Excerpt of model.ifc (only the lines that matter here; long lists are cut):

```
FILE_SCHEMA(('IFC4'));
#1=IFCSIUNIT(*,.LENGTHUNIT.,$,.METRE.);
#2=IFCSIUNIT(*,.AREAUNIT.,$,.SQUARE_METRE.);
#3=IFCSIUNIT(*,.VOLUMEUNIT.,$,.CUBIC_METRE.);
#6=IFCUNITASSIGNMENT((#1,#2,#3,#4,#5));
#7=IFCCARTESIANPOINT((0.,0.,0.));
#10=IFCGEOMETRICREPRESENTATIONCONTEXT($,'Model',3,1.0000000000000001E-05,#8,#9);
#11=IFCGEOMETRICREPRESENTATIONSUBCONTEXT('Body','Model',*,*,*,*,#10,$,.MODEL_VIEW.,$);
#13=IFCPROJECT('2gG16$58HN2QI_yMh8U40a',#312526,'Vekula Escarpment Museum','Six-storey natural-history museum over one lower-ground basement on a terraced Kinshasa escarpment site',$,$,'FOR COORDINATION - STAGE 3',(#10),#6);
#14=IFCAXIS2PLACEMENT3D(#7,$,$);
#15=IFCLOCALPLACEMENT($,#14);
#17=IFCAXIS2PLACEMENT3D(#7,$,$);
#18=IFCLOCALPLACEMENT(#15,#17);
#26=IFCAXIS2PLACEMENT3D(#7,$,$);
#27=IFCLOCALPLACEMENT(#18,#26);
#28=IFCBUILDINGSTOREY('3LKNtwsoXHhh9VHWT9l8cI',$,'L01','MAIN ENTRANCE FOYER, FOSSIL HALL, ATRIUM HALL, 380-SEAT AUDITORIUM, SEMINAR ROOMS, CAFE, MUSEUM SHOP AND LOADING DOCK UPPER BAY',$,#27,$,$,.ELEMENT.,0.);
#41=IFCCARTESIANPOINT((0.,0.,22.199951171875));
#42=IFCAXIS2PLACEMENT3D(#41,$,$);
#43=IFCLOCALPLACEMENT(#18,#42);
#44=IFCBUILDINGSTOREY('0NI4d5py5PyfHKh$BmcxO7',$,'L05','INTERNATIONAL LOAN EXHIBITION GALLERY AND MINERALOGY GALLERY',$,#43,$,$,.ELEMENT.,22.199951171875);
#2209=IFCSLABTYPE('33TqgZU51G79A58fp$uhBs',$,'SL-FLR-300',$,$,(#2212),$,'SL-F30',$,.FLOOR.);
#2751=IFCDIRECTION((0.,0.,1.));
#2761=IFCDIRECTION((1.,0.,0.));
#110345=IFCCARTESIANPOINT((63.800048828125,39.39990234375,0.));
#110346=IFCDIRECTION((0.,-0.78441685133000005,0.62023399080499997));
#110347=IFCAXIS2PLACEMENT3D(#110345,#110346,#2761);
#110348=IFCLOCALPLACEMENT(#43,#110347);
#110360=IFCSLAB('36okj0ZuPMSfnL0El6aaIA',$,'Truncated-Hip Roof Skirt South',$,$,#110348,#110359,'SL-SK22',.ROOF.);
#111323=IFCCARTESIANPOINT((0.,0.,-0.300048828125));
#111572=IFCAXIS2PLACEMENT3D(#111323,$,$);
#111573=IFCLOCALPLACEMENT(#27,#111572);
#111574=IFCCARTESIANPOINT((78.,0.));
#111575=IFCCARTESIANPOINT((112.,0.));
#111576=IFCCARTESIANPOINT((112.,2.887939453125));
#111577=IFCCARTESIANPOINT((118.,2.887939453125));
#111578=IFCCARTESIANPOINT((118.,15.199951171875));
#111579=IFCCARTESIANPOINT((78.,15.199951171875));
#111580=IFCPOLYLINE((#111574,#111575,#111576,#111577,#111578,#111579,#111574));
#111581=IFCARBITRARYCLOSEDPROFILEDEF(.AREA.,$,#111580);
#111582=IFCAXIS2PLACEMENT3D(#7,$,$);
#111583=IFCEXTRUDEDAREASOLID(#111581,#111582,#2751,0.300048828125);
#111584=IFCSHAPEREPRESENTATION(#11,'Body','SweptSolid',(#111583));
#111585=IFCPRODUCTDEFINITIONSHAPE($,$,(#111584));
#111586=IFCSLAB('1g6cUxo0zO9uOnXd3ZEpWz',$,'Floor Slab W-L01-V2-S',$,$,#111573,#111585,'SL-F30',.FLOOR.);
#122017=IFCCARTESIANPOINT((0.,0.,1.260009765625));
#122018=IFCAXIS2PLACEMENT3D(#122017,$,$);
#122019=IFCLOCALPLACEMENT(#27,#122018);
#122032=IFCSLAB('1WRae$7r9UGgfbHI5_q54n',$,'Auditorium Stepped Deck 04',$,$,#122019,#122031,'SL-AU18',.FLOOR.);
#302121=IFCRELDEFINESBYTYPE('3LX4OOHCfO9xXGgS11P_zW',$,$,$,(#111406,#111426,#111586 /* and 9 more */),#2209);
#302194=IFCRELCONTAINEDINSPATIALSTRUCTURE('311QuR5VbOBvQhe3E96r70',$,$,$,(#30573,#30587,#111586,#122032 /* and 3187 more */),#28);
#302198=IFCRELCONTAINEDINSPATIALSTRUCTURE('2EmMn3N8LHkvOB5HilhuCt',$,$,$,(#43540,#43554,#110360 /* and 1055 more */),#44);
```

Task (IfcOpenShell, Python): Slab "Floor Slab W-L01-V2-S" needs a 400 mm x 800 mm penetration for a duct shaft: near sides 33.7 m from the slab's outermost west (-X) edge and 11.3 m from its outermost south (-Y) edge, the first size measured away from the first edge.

```python
import numpy as np
import ifcopenshell
import ifcopenshell.api.feature
import ifcopenshell.api.geometry
import ifcopenshell.api.root
import ifcopenshell.geom
import ifcopenshell.util.placement
import ifcopenshell.util.representation
import ifcopenshell.util.shape
import ifcopenshell.util.unit

model = ifcopenshell.open("model.ifc")
unit_scale = ifcopenshell.util.unit.calculate_unit_scale(model)
settings = ifcopenshell.geom.settings()


def volume(element):
    """Net volume in cubic metres, openings subtracted."""
    shape = ifcopenshell.geom.create_shape(settings, element)
    return ifcopenshell.util.shape.get_volume(shape.geometry)


slab = model.by_guid("1g6cUxo0zO9uOnXd3ZEpWz")
before = volume(slab)

# Extent in the slab's own axes, in metres. The edges named are its -X and -Y sides.
slab_shape = ifcopenshell.geom.create_shape(settings, slab)
vertices = ifcopenshell.util.shape.get_vertices(slab_shape.geometry)
x_min, y_min, bottom = vertices.min(axis=0)
top = vertices[:, 2].max()

opening = ifcopenshell.api.root.create_entity(model, ifc_class="IfcOpeningElement", name="Duct shaft opening", predefined_type="OPENING")
context = ifcopenshell.util.representation.get_context(model, "Model", "Body", "MODEL_VIEW")
width, depth = 0.4, 0.8
outline = [(0.0, 0.0), (width, 0.0), (width, depth), (0.0, depth), (0.0, 0.0)]
# Overshoot both faces by 50 mm so the cut is clean.
shape = ifcopenshell.api.geometry.add_slab_representation(
    model, context=context, depth=top - bottom + 0.1, polyline=outline
)
ifcopenshell.api.geometry.assign_representation(model, product=opening, representation=shape)

matrix = ifcopenshell.util.placement.get_local_placement(slab.ObjectPlacement)
matrix[:, 3] = matrix @ np.append(np.array([x_min + 33.7, y_min + 11.3, bottom - 0.05]) / unit_scale, 1.0)
ifcopenshell.api.geometry.edit_object_placement(model, product=opening, matrix=matrix, is_si=False)
ifcopenshell.api.feature.add_feature(model, feature=opening, element=slab)

after = volume(slab)

print(f"slab volume {before:.3f} -> {after:.3f} m3")

model.write("model_rev.ifc")
```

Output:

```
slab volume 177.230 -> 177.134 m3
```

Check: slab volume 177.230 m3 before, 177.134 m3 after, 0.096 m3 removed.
